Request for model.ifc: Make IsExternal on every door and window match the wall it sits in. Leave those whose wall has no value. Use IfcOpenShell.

First a look at what the model holds.

```python
import ifcopenshell
import ifcopenshell.util.element

model = ifcopenshell.open("model.ifc")
print(model.schema)
seen = {}
for e in model.by_type("IfcDoor") + model.by_type("IfcWindow"):
    if not e.FillsVoids:
        continue
    host = e.FillsVoids[0].RelatingOpeningElement.VoidsElements[0].RelatingBuildingElement
    own = ifcopenshell.util.element.get_pset(e, f"Pset_{e.is_a()[3:].removesuffix('StandardCase')}Common", "IsExternal")
    wall = ifcopenshell.util.element.get_pset(host, "Pset_WallCommon", "IsExternal")
    seen[e.is_a(), own, wall] = seen.get((e.is_a(), own, wall), 0) + 1
for (cls, own, wall), count in sorted(seen.items(), key=str):
    print(count, cls, "IsExternal:", own, "| host wall:", wall)
```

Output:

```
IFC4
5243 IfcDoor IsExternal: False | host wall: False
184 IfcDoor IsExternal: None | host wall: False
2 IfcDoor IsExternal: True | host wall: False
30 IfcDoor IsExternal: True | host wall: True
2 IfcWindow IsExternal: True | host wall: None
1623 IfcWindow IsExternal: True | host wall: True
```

```python
import ifcopenshell
import ifcopenshell.api.pset
import ifcopenshell.util.element

model = ifcopenshell.open("model.ifc")

count = 0
for ifc_class, pset_name in (("IfcDoor", "Pset_DoorCommon"), ("IfcWindow", "Pset_WindowCommon")):
    for e in model.by_type(ifc_class):
        if not e.FillsVoids:
            continue
        host = e.FillsVoids[0].RelatingOpeningElement.VoidsElements[0].RelatingBuildingElement
        external = ifcopenshell.util.element.get_pset(host, "Pset_WallCommon", "IsExternal")
        if external is None or ifcopenshell.util.element.get_pset(e, pset_name, "IsExternal") == external:
            continue
        found = ifcopenshell.util.element.get_pset(e, pset_name, should_inherit=False)
        if found:
            pset = model.by_id(found["id"])
            if len(ifcopenshell.util.element.get_elements_by_pset(pset)) > 1:
                pset = ifcopenshell.api.pset.unshare_pset(model, products=[e], pset=pset)[0]
        else:
            pset = ifcopenshell.api.pset.add_pset(model, product=e, name=pset_name)
        ifcopenshell.api.pset.edit_pset(model, pset=pset, properties={"IsExternal": external})
        count += 1

print(count, "updated")

model.write("model_rev.ifc")
```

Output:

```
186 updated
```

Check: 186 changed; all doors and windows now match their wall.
